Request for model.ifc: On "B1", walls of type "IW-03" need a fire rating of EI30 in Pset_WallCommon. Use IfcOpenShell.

First a look at what the model holds.

```python
import ifcopenshell
import ifcopenshell.util.element

model = ifcopenshell.open("model.ifc")
print(model.schema)
storey = next(s for s in model.by_type("IfcBuildingStorey") if s.Name == "B1")
walls = [e for e in ifcopenshell.util.element.get_decomposition(storey) if e.is_a("IfcWall")]
seen = {}
for e in walls:
    element_type = ifcopenshell.util.element.get_type(e)
    key = (element_type.Name if element_type != e and element_type else None, ifcopenshell.util.element.get_pset(e, "Pset_WallCommon", "FireRating"))
    seen[key] = seen.get(key, 0) + 1
for (name, value), count in sorted(seen.items(), key=str):
    print(count, "x", name, "|", value)
```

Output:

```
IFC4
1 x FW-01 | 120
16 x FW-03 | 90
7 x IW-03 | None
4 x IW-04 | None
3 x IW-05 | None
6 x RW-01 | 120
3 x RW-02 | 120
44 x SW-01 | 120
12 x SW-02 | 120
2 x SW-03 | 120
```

```python
import ifcopenshell
import ifcopenshell.api.pset
import ifcopenshell.util.element

model = ifcopenshell.open("model.ifc")

storey = next(s for s in model.by_type("IfcBuildingStorey") if s.Name == "B1")
walls = [e for e in ifcopenshell.util.element.get_decomposition(storey) if e.is_a("IfcWall")]

count = 0
for e in walls:
    element_type = ifcopenshell.util.element.get_type(e)
    if element_type in (None, e) or element_type.Name != "IW-03":
        continue
    # add_pset returns the element's existing set when there is one.
    pset = ifcopenshell.api.pset.add_pset(model, product=e, name="Pset_WallCommon")
    ifcopenshell.api.pset.edit_pset(model, pset=pset, properties={"FireRating": "EI30"})
    count += 1

print(count, "walls updated")

model.write("model_rev.ifc")
```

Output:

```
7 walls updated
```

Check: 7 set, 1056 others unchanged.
